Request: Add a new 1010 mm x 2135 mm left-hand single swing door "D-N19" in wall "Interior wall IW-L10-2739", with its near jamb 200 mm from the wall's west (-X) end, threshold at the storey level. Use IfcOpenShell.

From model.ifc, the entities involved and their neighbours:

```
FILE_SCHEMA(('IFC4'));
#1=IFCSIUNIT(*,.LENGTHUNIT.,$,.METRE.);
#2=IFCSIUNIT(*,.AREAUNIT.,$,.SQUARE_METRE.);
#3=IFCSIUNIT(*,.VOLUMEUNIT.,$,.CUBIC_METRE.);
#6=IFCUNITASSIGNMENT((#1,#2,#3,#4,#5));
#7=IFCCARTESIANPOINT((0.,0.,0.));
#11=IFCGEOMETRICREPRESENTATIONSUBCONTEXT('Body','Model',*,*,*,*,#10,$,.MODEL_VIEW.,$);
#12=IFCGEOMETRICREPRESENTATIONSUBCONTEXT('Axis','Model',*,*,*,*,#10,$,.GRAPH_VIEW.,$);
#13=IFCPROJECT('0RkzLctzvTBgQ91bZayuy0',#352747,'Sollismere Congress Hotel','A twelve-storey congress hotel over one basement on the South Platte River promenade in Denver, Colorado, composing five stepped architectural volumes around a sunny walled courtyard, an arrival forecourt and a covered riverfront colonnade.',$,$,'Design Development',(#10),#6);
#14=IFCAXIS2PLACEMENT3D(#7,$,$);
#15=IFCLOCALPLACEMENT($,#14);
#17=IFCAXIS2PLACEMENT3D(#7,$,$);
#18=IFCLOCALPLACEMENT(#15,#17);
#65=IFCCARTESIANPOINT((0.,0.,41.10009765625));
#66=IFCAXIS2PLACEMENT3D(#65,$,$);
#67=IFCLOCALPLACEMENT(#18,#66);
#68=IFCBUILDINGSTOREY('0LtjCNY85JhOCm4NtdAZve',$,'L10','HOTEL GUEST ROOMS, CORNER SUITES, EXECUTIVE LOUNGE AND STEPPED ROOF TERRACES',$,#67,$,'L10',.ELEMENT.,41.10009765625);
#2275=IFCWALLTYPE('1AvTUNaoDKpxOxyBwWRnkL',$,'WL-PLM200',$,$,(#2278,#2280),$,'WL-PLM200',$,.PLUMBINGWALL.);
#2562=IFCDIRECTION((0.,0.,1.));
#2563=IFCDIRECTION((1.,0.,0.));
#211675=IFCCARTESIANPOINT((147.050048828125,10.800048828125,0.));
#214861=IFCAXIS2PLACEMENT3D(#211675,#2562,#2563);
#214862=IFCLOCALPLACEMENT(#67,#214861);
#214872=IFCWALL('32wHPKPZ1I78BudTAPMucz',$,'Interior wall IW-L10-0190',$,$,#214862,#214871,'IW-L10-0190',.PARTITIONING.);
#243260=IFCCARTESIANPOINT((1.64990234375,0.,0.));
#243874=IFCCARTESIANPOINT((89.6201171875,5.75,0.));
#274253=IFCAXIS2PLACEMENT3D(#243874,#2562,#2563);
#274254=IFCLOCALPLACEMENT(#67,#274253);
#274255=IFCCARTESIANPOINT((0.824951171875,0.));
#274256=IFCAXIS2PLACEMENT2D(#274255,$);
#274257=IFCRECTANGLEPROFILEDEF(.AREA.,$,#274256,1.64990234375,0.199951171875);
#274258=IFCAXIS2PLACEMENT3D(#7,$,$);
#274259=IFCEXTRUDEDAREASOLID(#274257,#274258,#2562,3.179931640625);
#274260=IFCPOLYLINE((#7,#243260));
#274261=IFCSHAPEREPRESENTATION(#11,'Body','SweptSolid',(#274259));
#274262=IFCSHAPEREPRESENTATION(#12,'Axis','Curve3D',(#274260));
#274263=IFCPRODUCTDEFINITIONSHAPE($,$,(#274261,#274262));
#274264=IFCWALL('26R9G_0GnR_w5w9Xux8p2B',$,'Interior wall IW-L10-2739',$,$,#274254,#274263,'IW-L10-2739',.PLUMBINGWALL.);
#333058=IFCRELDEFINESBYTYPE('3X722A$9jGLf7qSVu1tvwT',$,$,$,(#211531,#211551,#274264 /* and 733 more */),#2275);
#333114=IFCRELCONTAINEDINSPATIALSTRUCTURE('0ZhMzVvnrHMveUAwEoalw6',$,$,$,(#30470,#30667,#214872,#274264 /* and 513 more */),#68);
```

```python
import numpy as np
import ifcopenshell
import ifcopenshell.api.feature
import ifcopenshell.api.geometry
import ifcopenshell.api.root
import ifcopenshell.api.spatial
import ifcopenshell.geom
import ifcopenshell.util.element
import ifcopenshell.util.placement
import ifcopenshell.util.representation
import ifcopenshell.util.shape
import ifcopenshell.util.unit

model = ifcopenshell.open("model.ifc")
unit_scale = ifcopenshell.util.unit.calculate_unit_scale(model)
settings = ifcopenshell.geom.settings()


def volume(element):
    """Net volume in cubic metres, openings subtracted."""
    shape = ifcopenshell.geom.create_shape(settings, element)
    return ifcopenshell.util.shape.get_volume(shape.geometry)


wall = model.by_guid("26R9G_0GnR_w5w9Xux8p2B")
storey = ifcopenshell.util.element.get_container(wall, ifc_class="IfcBuildingStorey")
context = ifcopenshell.util.representation.get_context(model, "Model", "Body", "MODEL_VIEW")
before = volume(wall)

width, height, from_end, sill = 1.01, 2.135, 0.2, 0.0  # metres

# The wall runs along its own X axis, and the end named is its -X end.
wall_shape = ifcopenshell.geom.create_shape(settings, wall)
x, y, z = ifcopenshell.util.shape.get_vertices(wall_shape.geometry).T
start = x.min() + from_end
face, thickness = float(y.min()), float(y.max() - y.min())
wall_matrix = ifcopenshell.util.placement.get_local_placement(wall.ObjectPlacement)
level = ifcopenshell.util.placement.get_local_placement(storey.ObjectPlacement)[2, 3]


def in_wall(x, y):
    """Placement at x, y metres in the wall's axes, at sill height."""
    matrix = wall_matrix.copy()
    matrix[:, 3] = wall_matrix @ np.array([x / unit_scale, y / unit_scale, 0.0, 1.0])
    matrix[2, 3] = level + sill / unit_scale
    return matrix


# Opening: a box that overshoots both wall faces by 50 mm.
opening = ifcopenshell.api.root.create_entity(model, ifc_class="IfcOpeningElement", predefined_type="OPENING")
box = ifcopenshell.api.geometry.add_wall_representation(
    model, context=context, length=width, height=height, thickness=thickness + 0.1
)
ifcopenshell.api.geometry.assign_representation(model, product=opening, representation=box)
ifcopenshell.api.geometry.edit_object_placement(model, product=opening, matrix=in_wall(start, face - 0.05), is_si=False)
ifcopenshell.api.feature.add_feature(model, feature=opening, element=wall)

door = ifcopenshell.api.root.create_entity(model, ifc_class="IfcDoor", name="D-N19", predefined_type="DOOR")
door.OverallWidth, door.OverallHeight = width / unit_scale, height / unit_scale
door.OperationType = "SINGLE_SWING_LEFT"
body = ifcopenshell.api.geometry.add_door_representation(
    model,
    context=context,
    overall_width=door.OverallWidth,
    overall_height=door.OverallHeight,
    operation_type="SINGLE_SWING_LEFT",
    lining_properties={"LiningDepth": thickness / unit_scale, "ThresholdDepth": thickness / unit_scale},
)
ifcopenshell.api.geometry.assign_representation(model, product=door, representation=body)
ifcopenshell.api.spatial.assign_container(model, products=[door], relating_structure=storey)
ifcopenshell.api.feature.add_filling(model, opening=opening, element=door)

# The lining spans the wall, so the door starts at the wall face.
ifcopenshell.api.geometry.edit_object_placement(model, product=door, matrix=in_wall(start, face), is_si=False)

after = volume(wall)

print(f"wall volume {before:.3f} -> {after:.3f} m3")

model.write("model_rev.ifc")
```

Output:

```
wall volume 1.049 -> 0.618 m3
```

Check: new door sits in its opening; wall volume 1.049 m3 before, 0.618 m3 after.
